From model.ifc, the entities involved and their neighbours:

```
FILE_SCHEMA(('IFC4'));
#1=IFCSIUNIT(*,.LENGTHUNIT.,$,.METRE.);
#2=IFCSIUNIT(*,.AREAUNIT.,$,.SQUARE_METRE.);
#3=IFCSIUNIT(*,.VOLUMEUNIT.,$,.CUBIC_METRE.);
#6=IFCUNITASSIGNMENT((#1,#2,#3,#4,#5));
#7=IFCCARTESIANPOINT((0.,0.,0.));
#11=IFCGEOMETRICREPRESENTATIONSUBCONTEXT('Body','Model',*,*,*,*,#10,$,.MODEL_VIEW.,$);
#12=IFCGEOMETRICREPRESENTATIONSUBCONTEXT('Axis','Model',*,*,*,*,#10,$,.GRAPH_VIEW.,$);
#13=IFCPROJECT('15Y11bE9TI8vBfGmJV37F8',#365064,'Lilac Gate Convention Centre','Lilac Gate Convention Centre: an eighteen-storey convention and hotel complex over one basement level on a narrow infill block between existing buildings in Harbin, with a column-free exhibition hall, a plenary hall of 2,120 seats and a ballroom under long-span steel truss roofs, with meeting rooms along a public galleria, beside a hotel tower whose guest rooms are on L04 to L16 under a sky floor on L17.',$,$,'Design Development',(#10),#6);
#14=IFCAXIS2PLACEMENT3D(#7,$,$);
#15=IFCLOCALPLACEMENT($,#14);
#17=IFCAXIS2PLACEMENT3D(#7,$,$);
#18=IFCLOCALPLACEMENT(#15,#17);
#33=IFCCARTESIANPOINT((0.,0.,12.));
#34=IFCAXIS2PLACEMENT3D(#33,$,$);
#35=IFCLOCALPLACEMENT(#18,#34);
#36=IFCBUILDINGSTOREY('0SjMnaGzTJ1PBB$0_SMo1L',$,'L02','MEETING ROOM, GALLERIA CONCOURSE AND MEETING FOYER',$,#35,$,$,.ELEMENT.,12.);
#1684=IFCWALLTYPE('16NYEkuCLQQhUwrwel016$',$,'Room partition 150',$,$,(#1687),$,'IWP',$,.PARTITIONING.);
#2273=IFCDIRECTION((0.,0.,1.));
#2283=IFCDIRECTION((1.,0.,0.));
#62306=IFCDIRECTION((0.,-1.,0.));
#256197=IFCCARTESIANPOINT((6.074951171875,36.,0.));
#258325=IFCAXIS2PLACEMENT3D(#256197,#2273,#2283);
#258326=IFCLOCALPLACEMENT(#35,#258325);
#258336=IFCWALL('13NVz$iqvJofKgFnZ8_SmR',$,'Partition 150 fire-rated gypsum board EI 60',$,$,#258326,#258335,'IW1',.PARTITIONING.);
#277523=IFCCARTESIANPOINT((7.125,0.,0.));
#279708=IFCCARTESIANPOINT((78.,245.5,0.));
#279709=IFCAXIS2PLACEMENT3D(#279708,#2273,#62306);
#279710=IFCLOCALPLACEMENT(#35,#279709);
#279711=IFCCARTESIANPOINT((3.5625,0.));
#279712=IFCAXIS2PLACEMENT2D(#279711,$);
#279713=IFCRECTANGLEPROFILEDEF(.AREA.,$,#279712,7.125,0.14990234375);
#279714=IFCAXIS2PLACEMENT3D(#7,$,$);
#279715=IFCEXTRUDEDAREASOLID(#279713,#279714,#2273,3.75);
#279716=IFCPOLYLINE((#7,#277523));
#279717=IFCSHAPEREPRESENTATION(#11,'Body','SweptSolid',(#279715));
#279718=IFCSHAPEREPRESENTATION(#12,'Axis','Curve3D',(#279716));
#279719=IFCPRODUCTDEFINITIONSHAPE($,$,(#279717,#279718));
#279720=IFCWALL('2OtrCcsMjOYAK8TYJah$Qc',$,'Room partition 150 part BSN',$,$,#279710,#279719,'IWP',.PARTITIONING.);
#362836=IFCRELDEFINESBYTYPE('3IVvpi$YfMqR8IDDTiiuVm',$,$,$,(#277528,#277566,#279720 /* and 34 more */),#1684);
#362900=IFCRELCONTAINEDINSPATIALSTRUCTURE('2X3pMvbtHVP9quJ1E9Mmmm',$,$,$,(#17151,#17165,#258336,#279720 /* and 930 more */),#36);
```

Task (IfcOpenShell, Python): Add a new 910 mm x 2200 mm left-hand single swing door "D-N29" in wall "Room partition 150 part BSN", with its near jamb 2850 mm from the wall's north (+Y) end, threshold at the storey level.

```python
import numpy as np
import ifcopenshell
import ifcopenshell.api.feature
import ifcopenshell.api.geometry
import ifcopenshell.api.root
import ifcopenshell.api.spatial
import ifcopenshell.geom
import ifcopenshell.util.element
import ifcopenshell.util.placement
import ifcopenshell.util.representation
import ifcopenshell.util.shape
import ifcopenshell.util.unit

model = ifcopenshell.open("model.ifc")
unit_scale = ifcopenshell.util.unit.calculate_unit_scale(model)
settings = ifcopenshell.geom.settings()


def volume(element):
    """Net volume in cubic metres, openings subtracted."""
    shape = ifcopenshell.geom.create_shape(settings, element)
    return ifcopenshell.util.shape.get_volume(shape.geometry)


wall = model.by_id(279720)
storey = ifcopenshell.util.element.get_container(wall, ifc_class="IfcBuildingStorey")
context = ifcopenshell.util.representation.get_context(model, "Model", "Body", "MODEL_VIEW")
before = volume(wall)

width, height, from_end, sill = 0.91, 2.2, 2.85, 0.0  # metres

# The wall runs along its own X axis, and the end named is its -X end.
wall_shape = ifcopenshell.geom.create_shape(settings, wall)
x, y, z = ifcopenshell.util.shape.get_vertices(wall_shape.geometry).T
start = x.min() + from_end
face, thickness = float(y.min()), float(y.max() - y.min())
wall_matrix = ifcopenshell.util.placement.get_local_placement(wall.ObjectPlacement)
level = ifcopenshell.util.placement.get_local_placement(storey.ObjectPlacement)[2, 3]


def in_wall(x, y):
    """Placement at x, y metres in the wall's axes, at sill height."""
    matrix = wall_matrix.copy()
    matrix[:, 3] = wall_matrix @ np.array([x / unit_scale, y / unit_scale, 0.0, 1.0])
    matrix[2, 3] = level + sill / unit_scale
    return matrix


# Opening: a box that overshoots both wall faces by 50 mm.
opening = ifcopenshell.api.root.create_entity(model, ifc_class="IfcOpeningElement", predefined_type="OPENING")
box = ifcopenshell.api.geometry.add_wall_representation(
    model, context=context, length=width, height=height, thickness=thickness + 0.1
)
ifcopenshell.api.geometry.assign_representation(model, product=opening, representation=box)
ifcopenshell.api.geometry.edit_object_placement(model, product=opening, matrix=in_wall(start, face - 0.05), is_si=False)
ifcopenshell.api.feature.add_feature(model, feature=opening, element=wall)

door = ifcopenshell.api.root.create_entity(model, ifc_class="IfcDoor", name="D-N29", predefined_type="DOOR")
door.OverallWidth, door.OverallHeight = width / unit_scale, height / unit_scale
door.OperationType = "SINGLE_SWING_LEFT"
body = ifcopenshell.api.geometry.add_door_representation(
    model,
    context=context,
    overall_width=door.OverallWidth,
    overall_height=door.OverallHeight,
    operation_type="SINGLE_SWING_LEFT",
    lining_properties={"LiningDepth": thickness / unit_scale, "ThresholdDepth": thickness / unit_scale},
)
ifcopenshell.api.geometry.assign_representation(model, product=door, representation=body)
ifcopenshell.api.spatial.assign_container(model, products=[door], relating_structure=storey)
ifcopenshell.api.feature.add_filling(model, opening=opening, element=door)

# The lining spans the wall, so the door starts at the wall face.
ifcopenshell.api.geometry.edit_object_placement(model, product=door, matrix=in_wall(start, face), is_si=False)

after = volume(wall)

print(f"wall volume {before:.3f} -> {after:.3f} m3")

model.write("model_rev.ifc")
```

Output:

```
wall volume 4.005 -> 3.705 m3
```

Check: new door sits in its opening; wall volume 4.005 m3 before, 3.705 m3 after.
